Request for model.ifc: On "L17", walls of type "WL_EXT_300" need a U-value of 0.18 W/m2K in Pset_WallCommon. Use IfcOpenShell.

First a look at what the model holds.

```python
import ifcopenshell
import ifcopenshell.util.element

model = ifcopenshell.open("model.ifc")
print(model.schema)
storey = next(s for s in model.by_type("IfcBuildingStorey") if s.Name == "L17")
walls = [e for e in ifcopenshell.util.element.get_decomposition(storey) if e.is_a("IfcWall")]
seen = {}
for e in walls:
    element_type = ifcopenshell.util.element.get_type(e)
    key = (element_type.Name if element_type != e and element_type else None, ifcopenshell.util.element.get_pset(e, "Pset_WallCommon", "ThermalTransmittance"))
    seen[key] = seen.get(key, 0) + 1
for (name, value), count in sorted(seen.items(), key=str):
    print(count, "x", name, "|", value)
```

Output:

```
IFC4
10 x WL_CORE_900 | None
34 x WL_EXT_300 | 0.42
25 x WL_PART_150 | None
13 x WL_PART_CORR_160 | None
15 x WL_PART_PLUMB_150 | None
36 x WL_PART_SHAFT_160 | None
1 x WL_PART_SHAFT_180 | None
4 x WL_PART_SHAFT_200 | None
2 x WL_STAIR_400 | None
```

```python
import ifcopenshell
import ifcopenshell.api.pset
import ifcopenshell.util.element

model = ifcopenshell.open("model.ifc")

storey = next(s for s in model.by_type("IfcBuildingStorey") if s.Name == "L17")
walls = [e for e in ifcopenshell.util.element.get_decomposition(storey) if e.is_a("IfcWall")]

count = 0
for e in walls:
    element_type = ifcopenshell.util.element.get_type(e)
    if element_type in (None, e) or element_type.Name != "WL_EXT_300":
        continue
    found = ifcopenshell.util.element.get_pset(e, "Pset_WallCommon", should_inherit=False)
    if found:
        pset = model.by_id(found["id"])
        if len(ifcopenshell.util.element.get_elements_by_pset(pset)) > 1:
            pset = ifcopenshell.api.pset.unshare_pset(model, products=[e], pset=pset)[0]
    else:
        pset = ifcopenshell.api.pset.add_pset(model, product=e, name="Pset_WallCommon")
    ifcopenshell.api.pset.edit_pset(model, pset=pset, properties={"ThermalTransmittance": 0.18})
    count += 1

print(count, "walls updated")

model.write("model_updated.ifc")
```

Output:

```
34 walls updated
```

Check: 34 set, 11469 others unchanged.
